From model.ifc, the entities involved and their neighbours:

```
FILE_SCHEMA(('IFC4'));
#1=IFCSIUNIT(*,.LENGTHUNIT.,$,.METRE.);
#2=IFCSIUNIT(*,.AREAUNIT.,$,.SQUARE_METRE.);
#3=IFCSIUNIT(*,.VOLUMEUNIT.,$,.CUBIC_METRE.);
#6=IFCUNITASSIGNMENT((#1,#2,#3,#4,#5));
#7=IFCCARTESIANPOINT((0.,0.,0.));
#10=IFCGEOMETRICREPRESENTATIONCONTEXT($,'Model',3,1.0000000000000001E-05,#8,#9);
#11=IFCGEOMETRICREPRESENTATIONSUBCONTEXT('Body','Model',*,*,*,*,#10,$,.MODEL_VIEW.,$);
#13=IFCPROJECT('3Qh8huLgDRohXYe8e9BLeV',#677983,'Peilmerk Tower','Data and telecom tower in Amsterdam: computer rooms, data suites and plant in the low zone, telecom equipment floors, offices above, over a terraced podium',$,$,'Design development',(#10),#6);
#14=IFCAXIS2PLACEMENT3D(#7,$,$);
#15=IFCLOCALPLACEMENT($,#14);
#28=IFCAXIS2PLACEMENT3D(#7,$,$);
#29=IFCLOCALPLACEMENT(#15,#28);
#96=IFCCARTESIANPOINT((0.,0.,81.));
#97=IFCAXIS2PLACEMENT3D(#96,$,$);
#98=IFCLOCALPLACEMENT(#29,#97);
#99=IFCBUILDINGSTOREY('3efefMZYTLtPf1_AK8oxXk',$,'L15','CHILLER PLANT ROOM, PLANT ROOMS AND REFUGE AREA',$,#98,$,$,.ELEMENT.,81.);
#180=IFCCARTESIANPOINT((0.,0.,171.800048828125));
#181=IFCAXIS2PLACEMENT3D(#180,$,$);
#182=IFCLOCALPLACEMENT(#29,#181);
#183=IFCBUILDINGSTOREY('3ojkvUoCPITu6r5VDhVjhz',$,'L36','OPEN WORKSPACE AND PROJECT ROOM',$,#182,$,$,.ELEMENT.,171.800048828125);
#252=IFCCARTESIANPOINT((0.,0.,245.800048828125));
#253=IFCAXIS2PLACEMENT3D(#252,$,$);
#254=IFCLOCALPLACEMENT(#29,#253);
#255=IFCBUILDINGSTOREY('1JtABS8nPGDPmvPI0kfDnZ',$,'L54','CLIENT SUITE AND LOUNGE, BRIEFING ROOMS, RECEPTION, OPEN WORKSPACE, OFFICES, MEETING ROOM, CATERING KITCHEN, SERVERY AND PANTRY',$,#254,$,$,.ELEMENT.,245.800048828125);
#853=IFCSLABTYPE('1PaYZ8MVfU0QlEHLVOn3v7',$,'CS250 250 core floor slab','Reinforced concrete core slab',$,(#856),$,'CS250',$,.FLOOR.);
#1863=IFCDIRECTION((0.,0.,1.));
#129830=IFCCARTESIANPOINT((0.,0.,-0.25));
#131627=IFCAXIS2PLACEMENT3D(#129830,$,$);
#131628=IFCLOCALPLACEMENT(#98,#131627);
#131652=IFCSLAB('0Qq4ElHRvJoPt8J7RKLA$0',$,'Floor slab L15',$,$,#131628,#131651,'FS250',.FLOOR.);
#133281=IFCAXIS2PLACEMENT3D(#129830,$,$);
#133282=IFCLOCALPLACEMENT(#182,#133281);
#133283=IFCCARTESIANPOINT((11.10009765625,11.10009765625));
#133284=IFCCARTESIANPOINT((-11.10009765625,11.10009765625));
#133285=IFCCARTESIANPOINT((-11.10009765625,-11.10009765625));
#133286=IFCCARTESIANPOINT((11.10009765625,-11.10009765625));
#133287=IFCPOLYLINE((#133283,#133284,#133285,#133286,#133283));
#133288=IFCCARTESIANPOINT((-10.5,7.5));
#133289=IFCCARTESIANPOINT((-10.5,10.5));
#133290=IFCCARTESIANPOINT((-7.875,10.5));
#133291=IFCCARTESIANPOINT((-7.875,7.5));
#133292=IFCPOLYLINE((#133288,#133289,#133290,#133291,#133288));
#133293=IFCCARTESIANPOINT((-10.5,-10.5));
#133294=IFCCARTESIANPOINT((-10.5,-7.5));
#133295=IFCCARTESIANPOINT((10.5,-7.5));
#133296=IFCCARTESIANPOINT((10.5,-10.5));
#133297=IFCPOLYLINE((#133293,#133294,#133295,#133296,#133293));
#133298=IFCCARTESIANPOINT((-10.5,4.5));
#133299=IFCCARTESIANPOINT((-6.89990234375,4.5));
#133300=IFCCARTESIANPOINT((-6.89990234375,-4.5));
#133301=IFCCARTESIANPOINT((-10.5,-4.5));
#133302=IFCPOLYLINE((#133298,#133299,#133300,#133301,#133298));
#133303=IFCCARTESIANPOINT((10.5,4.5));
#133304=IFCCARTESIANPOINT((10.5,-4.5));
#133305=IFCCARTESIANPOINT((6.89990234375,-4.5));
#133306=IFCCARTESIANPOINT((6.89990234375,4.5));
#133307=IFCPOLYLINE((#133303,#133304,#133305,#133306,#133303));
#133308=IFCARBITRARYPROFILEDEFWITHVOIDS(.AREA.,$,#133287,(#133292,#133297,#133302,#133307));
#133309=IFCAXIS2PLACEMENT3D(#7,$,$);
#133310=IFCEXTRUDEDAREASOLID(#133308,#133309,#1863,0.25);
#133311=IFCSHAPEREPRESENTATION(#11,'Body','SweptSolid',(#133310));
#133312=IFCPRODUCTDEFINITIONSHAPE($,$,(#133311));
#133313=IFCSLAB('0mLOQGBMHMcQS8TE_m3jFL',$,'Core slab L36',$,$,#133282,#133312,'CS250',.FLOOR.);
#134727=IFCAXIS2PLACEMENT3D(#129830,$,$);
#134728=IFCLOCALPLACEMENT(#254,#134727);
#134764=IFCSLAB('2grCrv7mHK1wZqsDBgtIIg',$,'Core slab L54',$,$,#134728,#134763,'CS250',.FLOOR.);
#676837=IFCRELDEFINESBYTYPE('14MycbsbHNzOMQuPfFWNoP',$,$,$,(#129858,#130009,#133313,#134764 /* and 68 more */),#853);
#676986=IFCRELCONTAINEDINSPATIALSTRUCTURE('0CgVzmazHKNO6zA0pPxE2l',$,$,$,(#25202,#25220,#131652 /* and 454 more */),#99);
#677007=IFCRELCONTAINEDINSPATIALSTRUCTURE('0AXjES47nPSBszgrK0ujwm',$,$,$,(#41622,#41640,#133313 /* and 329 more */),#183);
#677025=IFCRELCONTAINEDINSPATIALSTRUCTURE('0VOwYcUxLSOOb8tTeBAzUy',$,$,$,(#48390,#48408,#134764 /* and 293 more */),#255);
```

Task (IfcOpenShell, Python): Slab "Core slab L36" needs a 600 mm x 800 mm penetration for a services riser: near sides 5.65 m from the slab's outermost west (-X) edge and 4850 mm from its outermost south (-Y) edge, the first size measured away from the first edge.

```python
import numpy as np
import ifcopenshell
import ifcopenshell.api.feature
import ifcopenshell.api.geometry
import ifcopenshell.api.root
import ifcopenshell.geom
import ifcopenshell.util.placement
import ifcopenshell.util.representation
import ifcopenshell.util.shape
import ifcopenshell.util.unit

model = ifcopenshell.open("model.ifc")
unit_scale = ifcopenshell.util.unit.calculate_unit_scale(model)
settings = ifcopenshell.geom.settings()


def volume(element):
    """Net volume in cubic metres, openings subtracted."""
    shape = ifcopenshell.geom.create_shape(settings, element)
    return ifcopenshell.util.shape.get_volume(shape.geometry)


slab = model.by_id(133313)
before = volume(slab)

# Extent in the slab's own axes, in metres. The edges named are its -X and -Y sides.
slab_shape = ifcopenshell.geom.create_shape(settings, slab)
vertices = ifcopenshell.util.shape.get_vertices(slab_shape.geometry)
x_min, y_min, bottom = vertices.min(axis=0)
top = vertices[:, 2].max()

opening = ifcopenshell.api.root.create_entity(model, ifc_class="IfcOpeningElement", name="Services riser opening", predefined_type="OPENING")
context = ifcopenshell.util.representation.get_context(model, "Model", "Body", "MODEL_VIEW")
width, depth = 0.6, 0.8
outline = [(0.0, 0.0), (width, 0.0), (width, depth), (0.0, depth), (0.0, 0.0)]
# Overshoot both faces by 50 mm so the cut is clean.
shape = ifcopenshell.api.geometry.add_slab_representation(
    model, context=context, depth=top - bottom + 0.1, polyline=outline
)
ifcopenshell.api.geometry.assign_representation(model, product=opening, representation=shape)

matrix = ifcopenshell.util.placement.get_local_placement(slab.ObjectPlacement)
matrix[:, 3] = matrix @ np.append(np.array([x_min + 5.65, y_min + 4.85, bottom - 0.05]) / unit_scale, 1.0)
ifcopenshell.api.geometry.edit_object_placement(model, product=opening, matrix=matrix, is_si=False)
ifcopenshell.api.feature.add_feature(model, feature=opening, element=slab)

after = volume(slab)

print(f"slab volume {before:.3f} -> {after:.3f} m3")

model.write("model_updated.ifc")
```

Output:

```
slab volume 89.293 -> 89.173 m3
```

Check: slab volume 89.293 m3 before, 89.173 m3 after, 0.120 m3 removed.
